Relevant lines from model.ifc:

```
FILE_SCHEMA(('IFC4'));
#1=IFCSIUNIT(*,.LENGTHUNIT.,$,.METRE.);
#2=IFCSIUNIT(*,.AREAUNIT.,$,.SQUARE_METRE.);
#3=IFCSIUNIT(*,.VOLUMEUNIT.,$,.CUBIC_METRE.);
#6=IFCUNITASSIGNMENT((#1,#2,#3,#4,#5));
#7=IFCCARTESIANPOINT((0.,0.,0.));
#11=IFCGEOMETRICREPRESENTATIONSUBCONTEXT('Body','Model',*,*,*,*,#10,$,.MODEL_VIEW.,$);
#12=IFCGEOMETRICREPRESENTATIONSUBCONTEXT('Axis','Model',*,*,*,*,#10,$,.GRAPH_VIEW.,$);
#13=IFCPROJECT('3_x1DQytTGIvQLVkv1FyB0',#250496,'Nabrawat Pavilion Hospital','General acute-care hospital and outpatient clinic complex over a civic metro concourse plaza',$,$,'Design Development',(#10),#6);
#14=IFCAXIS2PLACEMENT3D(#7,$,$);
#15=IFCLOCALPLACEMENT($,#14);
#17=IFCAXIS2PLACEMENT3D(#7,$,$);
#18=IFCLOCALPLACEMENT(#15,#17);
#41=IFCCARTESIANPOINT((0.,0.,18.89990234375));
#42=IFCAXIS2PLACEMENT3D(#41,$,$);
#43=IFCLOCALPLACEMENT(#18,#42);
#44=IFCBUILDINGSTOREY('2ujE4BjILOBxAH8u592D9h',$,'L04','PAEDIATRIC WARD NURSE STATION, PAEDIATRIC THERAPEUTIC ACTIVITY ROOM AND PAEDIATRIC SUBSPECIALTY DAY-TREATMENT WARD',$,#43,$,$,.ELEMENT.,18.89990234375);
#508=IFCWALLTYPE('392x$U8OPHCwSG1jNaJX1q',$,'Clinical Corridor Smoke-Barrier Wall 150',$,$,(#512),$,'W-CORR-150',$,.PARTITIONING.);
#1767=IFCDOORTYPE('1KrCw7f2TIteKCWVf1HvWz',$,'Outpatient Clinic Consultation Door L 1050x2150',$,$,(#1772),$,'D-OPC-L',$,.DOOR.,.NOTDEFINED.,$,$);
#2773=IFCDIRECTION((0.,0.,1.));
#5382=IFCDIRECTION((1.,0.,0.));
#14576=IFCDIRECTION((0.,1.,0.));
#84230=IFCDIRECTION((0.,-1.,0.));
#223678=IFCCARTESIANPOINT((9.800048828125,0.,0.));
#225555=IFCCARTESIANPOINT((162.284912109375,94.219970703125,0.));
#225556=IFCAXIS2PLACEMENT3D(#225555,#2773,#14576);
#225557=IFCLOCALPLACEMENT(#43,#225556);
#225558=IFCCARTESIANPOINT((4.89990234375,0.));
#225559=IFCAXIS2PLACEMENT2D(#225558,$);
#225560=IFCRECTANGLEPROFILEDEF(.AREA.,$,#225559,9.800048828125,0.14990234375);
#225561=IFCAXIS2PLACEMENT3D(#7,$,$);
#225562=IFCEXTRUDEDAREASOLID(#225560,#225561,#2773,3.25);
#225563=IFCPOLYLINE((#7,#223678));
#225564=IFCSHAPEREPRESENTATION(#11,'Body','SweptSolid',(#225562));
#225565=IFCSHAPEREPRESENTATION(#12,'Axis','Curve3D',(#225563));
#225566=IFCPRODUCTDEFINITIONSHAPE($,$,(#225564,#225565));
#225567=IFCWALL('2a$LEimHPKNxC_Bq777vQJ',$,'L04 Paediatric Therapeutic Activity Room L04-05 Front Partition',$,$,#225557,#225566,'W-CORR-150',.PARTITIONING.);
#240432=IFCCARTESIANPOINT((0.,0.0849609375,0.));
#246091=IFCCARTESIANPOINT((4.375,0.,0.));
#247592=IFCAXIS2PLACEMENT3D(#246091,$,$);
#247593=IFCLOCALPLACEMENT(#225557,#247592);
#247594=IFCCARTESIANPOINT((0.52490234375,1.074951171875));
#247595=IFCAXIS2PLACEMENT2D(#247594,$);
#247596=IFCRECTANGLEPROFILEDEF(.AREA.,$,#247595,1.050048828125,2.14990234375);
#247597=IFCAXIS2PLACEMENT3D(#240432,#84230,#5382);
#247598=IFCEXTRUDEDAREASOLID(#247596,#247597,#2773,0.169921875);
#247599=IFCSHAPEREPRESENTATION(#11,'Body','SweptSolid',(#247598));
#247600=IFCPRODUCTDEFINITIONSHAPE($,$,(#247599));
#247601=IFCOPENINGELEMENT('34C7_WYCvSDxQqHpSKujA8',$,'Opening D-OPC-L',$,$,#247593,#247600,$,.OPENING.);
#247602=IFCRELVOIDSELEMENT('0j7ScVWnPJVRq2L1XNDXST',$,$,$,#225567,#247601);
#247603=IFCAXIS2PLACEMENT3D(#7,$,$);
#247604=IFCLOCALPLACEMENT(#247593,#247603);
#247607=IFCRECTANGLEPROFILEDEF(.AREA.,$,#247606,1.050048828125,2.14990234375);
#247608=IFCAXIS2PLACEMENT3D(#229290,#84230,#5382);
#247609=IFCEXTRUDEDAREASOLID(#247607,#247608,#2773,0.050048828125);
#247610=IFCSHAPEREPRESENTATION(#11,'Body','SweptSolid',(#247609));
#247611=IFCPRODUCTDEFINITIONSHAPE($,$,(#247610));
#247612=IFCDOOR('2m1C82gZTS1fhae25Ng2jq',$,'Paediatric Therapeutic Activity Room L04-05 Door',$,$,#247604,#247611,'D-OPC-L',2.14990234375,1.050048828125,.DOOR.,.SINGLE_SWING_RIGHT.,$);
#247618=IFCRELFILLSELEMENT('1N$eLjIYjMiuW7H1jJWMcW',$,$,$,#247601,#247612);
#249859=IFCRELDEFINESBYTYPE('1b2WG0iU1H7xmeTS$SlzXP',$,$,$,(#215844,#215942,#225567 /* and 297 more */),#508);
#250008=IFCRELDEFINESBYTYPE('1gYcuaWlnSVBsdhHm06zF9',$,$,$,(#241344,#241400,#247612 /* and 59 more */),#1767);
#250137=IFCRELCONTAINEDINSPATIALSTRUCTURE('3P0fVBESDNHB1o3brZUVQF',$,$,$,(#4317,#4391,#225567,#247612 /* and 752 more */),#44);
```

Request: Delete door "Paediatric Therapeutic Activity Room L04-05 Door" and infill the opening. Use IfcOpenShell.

```python
import ifcopenshell
import ifcopenshell.api.feature
import ifcopenshell.api.root
import ifcopenshell.geom
import ifcopenshell.util.shape

model = ifcopenshell.open("model.ifc")
settings = ifcopenshell.geom.settings()


def volume(element):
    """Net volume in cubic metres, openings subtracted."""
    shape = ifcopenshell.geom.create_shape(settings, element)
    return ifcopenshell.util.shape.get_volume(shape.geometry)


door = model.by_guid("2m1C82gZTS1fhae25Ng2jq")
opening = door.FillsVoids[0].RelatingOpeningElement
wall = opening.VoidsElements[0].RelatingBuildingElement
before = volume(wall)

ifcopenshell.api.root.remove_product(model, product=door)
ifcopenshell.api.feature.remove_feature(model, feature=opening)

after = volume(wall)

print(f"wall volume {before:.3f} -> {after:.3f} m3")

model.write("model_updated.ifc")
```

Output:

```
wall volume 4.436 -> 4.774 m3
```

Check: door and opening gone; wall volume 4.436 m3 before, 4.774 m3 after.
